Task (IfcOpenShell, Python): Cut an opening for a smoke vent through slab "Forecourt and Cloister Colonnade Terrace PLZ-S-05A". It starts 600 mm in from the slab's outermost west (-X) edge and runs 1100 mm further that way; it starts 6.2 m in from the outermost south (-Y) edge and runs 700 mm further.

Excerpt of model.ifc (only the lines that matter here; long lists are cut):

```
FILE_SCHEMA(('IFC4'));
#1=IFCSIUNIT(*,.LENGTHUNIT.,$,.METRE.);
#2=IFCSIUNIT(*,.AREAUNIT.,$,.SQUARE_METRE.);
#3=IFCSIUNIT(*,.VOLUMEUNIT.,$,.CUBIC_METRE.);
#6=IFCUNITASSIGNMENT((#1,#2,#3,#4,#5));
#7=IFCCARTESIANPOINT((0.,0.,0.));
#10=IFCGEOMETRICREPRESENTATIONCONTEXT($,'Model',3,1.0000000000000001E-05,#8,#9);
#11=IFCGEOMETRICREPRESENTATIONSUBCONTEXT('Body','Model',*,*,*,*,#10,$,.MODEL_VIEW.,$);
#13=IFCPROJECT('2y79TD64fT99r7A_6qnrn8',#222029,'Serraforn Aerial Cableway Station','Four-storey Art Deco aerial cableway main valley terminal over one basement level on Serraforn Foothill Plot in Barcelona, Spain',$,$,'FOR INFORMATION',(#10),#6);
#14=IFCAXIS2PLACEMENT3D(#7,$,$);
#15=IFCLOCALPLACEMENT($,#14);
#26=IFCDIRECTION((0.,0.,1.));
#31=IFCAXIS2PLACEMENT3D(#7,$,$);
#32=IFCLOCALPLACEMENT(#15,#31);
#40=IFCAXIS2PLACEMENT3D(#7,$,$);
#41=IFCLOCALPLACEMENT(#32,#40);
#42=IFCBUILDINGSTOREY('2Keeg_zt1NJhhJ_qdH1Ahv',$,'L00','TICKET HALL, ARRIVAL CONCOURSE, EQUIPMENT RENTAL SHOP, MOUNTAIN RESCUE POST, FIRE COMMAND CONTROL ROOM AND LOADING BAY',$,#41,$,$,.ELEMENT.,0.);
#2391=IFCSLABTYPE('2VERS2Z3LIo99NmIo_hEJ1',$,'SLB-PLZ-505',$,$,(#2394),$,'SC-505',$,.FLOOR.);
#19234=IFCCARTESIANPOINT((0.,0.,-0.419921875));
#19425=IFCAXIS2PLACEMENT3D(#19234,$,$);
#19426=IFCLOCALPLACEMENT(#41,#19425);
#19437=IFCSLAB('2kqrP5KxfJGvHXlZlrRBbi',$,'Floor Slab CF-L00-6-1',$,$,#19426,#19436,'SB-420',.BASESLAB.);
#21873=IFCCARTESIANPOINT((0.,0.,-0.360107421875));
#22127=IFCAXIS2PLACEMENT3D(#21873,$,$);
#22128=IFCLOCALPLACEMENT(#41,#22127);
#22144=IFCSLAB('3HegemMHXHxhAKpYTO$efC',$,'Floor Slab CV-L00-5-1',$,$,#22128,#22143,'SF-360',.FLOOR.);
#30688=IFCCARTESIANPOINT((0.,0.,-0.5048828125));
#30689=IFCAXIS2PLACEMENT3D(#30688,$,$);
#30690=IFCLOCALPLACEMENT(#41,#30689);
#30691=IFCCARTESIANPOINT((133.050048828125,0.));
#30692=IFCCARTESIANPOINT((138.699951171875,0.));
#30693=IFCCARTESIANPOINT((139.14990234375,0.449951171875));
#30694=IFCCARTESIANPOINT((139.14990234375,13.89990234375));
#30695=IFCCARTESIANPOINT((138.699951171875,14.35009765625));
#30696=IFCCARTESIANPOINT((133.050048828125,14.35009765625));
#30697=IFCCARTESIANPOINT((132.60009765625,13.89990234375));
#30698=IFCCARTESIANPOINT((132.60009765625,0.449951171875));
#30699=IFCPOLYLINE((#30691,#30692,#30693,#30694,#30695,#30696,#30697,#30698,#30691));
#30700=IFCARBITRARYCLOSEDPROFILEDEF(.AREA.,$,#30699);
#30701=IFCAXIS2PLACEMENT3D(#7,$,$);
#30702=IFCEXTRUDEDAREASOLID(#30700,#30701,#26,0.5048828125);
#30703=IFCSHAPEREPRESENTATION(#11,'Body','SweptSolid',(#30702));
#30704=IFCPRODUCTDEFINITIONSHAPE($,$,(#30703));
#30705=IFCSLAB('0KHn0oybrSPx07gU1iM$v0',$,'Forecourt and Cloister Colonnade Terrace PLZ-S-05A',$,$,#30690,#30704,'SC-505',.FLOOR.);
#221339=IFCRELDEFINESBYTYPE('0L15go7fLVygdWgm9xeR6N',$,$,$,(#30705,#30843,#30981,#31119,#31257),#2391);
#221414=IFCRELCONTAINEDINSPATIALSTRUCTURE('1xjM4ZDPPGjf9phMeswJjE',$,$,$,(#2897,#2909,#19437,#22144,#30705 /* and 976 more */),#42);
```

```python
import numpy as np
import ifcopenshell
import ifcopenshell.api.feature
import ifcopenshell.api.geometry
import ifcopenshell.api.root
import ifcopenshell.geom
import ifcopenshell.util.placement
import ifcopenshell.util.representation
import ifcopenshell.util.shape
import ifcopenshell.util.unit

model = ifcopenshell.open("model.ifc")
unit_scale = ifcopenshell.util.unit.calculate_unit_scale(model)
settings = ifcopenshell.geom.settings()


def volume(element):
    """Net volume in cubic metres, openings subtracted."""
    shape = ifcopenshell.geom.create_shape(settings, element)
    return ifcopenshell.util.shape.get_volume(shape.geometry)


slab = model.by_id(30705)
before = volume(slab)

# Extent in the slab's own axes, in metres. The edges named are its -X and -Y sides.
slab_shape = ifcopenshell.geom.create_shape(settings, slab)
vertices = ifcopenshell.util.shape.get_vertices(slab_shape.geometry)
x_min, y_min, bottom = vertices.min(axis=0)
top = vertices[:, 2].max()

opening = ifcopenshell.api.root.create_entity(model, ifc_class="IfcOpeningElement", name="Smoke vent opening", predefined_type="OPENING")
context = ifcopenshell.util.representation.get_context(model, "Model", "Body", "MODEL_VIEW")
width, depth = 1.1, 0.7
outline = [(0.0, 0.0), (width, 0.0), (width, depth), (0.0, depth), (0.0, 0.0)]
# Overshoot both faces by 50 mm so the cut is clean.
shape = ifcopenshell.api.geometry.add_slab_representation(
    model, context=context, depth=top - bottom + 0.1, polyline=outline
)
ifcopenshell.api.geometry.assign_representation(model, product=opening, representation=shape)

matrix = ifcopenshell.util.placement.get_local_placement(slab.ObjectPlacement)
matrix[:, 3] = matrix @ np.append(np.array([x_min + 0.6, y_min + 6.2, bottom - 0.05]) / unit_scale, 1.0)
ifcopenshell.api.geometry.edit_object_placement(model, product=opening, matrix=matrix, is_si=False)
ifcopenshell.api.feature.add_feature(model, feature=opening, element=slab)

after = volume(slab)

print(f"slab volume {before:.3f} -> {after:.3f} m3")

model.write("model_rev.ifc")
```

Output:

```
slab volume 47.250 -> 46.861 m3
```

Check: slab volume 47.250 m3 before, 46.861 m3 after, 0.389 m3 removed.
